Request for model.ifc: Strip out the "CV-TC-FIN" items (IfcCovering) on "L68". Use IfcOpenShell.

First a look at what the model holds.

```python
import ifcopenshell
import ifcopenshell.util.element

model = ifcopenshell.open("model.ifc")
print(model.schema)
storey = next(s for s in model.by_type("IfcBuildingStorey") if s.Name == "L68")
coverings = [e for e in ifcopenshell.util.element.get_decomposition(storey) if e.is_a("IfcCovering")]
seen = {}
for e in coverings:
    element_type = ifcopenshell.util.element.get_type(e)
    name = element_type.Name if element_type not in (None, e) else None
    seen[name] = seen.get(name, 0) + 1
for name, count in sorted(seen.items(), key=str):
    print(count, "x", name)
```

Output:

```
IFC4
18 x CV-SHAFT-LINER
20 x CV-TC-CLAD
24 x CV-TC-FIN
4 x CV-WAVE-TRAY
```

```python
import ifcopenshell
import ifcopenshell.api.root
import ifcopenshell.util.element

model = ifcopenshell.open("model.ifc")

storey = next(s for s in model.by_type("IfcBuildingStorey") if s.Name == "L68")
coverings = [e for e in ifcopenshell.util.element.get_decomposition(storey) if e.is_a("IfcCovering")]
targets = [e for e in coverings if (t := ifcopenshell.util.element.get_type(e)) not in (None, e) and t.Name == "CV-TC-FIN"]

for e in targets:
    ifcopenshell.api.root.remove_product(model, product=e)
print(len(targets), "removed")

model.write("model_edited.ifc")
```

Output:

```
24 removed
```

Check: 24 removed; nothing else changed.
